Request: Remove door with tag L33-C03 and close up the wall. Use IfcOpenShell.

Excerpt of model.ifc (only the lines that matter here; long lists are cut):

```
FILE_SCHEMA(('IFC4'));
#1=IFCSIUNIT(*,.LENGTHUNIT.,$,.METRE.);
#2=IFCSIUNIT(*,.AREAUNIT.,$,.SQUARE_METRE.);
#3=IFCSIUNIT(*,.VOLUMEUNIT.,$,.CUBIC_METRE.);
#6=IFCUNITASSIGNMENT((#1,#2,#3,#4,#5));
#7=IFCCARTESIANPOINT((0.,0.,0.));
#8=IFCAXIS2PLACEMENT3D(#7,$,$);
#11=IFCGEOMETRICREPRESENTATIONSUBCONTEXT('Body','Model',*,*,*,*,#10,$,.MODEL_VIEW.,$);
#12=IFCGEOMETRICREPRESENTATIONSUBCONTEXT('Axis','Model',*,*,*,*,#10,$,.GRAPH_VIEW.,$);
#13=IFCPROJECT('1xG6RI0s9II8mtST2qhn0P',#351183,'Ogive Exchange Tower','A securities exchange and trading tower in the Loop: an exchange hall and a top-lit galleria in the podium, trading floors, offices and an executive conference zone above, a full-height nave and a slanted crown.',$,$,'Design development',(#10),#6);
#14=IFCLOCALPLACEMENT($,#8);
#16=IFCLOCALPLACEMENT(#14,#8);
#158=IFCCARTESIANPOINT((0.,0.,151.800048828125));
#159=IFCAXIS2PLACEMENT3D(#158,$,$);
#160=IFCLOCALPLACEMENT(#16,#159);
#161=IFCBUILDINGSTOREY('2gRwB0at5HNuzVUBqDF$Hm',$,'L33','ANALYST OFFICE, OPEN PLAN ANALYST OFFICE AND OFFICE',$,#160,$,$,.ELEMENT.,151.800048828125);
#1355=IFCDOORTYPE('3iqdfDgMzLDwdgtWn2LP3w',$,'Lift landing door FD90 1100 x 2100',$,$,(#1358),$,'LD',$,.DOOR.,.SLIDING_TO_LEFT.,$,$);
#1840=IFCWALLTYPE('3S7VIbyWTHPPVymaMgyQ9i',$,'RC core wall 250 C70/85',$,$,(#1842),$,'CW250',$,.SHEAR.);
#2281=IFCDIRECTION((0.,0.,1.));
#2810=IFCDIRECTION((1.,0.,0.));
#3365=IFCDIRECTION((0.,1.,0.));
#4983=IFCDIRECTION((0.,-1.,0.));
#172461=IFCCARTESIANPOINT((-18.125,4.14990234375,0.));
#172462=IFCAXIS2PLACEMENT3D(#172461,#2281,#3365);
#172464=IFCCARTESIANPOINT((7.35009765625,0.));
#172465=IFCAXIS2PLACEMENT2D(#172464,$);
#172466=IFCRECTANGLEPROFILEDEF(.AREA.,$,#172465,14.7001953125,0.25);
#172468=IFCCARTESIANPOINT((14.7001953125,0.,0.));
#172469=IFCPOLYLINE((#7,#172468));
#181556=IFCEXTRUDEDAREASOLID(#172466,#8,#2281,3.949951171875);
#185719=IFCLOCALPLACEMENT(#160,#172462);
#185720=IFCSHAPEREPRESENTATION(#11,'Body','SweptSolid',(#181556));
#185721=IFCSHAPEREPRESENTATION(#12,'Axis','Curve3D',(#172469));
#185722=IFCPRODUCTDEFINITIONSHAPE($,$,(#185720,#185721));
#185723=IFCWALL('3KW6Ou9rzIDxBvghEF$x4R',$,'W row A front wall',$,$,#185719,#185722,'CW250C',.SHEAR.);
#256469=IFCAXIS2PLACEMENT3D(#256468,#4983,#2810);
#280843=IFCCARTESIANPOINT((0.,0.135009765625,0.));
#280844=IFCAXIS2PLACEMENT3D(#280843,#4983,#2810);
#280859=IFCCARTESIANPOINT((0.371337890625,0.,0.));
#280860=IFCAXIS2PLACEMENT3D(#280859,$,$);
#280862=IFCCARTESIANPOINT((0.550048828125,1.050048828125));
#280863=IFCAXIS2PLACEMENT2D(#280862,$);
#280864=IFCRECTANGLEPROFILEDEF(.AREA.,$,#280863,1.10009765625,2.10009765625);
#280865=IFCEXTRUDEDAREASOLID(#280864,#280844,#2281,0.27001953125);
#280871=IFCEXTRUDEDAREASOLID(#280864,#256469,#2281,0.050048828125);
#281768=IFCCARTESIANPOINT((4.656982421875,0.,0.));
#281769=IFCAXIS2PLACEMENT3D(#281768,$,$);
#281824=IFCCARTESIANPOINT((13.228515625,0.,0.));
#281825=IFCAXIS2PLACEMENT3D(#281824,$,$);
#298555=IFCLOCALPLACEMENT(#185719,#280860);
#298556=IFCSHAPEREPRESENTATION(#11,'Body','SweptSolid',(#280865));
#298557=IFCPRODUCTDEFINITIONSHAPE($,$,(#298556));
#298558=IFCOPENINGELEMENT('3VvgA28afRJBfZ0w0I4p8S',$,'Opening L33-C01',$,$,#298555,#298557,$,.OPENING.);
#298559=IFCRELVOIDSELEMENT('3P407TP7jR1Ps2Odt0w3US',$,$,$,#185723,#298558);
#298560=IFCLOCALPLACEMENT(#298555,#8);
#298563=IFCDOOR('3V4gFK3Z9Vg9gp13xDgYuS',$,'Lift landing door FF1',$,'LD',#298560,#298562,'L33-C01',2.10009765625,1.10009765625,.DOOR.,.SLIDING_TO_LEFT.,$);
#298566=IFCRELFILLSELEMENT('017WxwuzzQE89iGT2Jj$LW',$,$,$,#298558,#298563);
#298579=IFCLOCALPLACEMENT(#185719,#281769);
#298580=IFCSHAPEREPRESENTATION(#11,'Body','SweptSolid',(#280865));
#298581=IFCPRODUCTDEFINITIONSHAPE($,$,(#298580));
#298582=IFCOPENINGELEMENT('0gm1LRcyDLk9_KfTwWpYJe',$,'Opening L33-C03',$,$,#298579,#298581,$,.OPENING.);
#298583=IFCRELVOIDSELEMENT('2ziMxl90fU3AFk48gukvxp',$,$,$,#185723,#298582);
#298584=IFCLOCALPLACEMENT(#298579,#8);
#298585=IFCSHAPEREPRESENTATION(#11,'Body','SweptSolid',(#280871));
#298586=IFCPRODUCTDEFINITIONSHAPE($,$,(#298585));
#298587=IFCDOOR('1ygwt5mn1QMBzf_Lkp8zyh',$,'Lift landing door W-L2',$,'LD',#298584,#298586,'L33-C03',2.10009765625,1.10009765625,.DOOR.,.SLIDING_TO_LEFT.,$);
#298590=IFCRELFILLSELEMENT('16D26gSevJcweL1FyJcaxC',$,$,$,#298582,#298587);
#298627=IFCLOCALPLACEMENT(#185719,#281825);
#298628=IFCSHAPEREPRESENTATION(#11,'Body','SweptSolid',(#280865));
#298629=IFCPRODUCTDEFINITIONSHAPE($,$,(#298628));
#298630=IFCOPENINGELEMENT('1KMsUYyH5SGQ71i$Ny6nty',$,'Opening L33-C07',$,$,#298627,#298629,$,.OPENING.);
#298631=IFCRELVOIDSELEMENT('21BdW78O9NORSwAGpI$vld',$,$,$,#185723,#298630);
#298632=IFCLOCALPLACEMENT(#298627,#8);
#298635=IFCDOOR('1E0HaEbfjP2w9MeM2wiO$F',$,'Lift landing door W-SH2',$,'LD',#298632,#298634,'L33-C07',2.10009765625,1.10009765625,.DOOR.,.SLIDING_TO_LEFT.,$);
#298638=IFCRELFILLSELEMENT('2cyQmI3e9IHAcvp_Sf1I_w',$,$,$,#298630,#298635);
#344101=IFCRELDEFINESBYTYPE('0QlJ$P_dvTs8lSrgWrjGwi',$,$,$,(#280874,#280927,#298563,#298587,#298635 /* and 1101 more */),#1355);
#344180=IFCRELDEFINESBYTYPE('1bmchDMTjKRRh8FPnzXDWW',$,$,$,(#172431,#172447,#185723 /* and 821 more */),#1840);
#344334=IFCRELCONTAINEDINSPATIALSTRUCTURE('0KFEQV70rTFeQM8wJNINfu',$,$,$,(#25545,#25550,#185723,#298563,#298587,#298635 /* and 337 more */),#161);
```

```python
import ifcopenshell
import ifcopenshell.api.feature
import ifcopenshell.api.root
import ifcopenshell.geom
import ifcopenshell.util.shape

model = ifcopenshell.open("model.ifc")
settings = ifcopenshell.geom.settings()


def volume(element):
    """Net volume in cubic metres, openings subtracted."""
    shape = ifcopenshell.geom.create_shape(settings, element)
    return ifcopenshell.util.shape.get_volume(shape.geometry)


door = model.by_guid("1ygwt5mn1QMBzf_Lkp8zyh")
opening = door.FillsVoids[0].RelatingOpeningElement
wall = opening.VoidsElements[0].RelatingBuildingElement
before = volume(wall)

ifcopenshell.api.root.remove_product(model, product=door)
ifcopenshell.api.feature.remove_feature(model, feature=opening)

after = volume(wall)

print(f"wall volume {before:.3f} -> {after:.3f} m3")

model.write("model-out.ifc")
```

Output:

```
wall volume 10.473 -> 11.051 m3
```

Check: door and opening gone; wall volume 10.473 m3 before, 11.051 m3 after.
